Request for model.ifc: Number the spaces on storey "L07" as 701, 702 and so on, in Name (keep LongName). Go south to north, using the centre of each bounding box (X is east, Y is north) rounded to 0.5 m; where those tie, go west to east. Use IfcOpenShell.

First a look at what the model holds.

```python
import ifcopenshell
import ifcopenshell.util.element
import ifcopenshell.util.placement

model = ifcopenshell.open("model.ifc")
print(model.schema)
storey = next(s for s in model.by_type("IfcBuildingStorey") if s.Name == "L07")
spaces = [e for e in ifcopenshell.util.element.get_decomposition(storey) if e.is_a("IfcSpace")]
for e in sorted(spaces, key=lambda e: e.id()):
    origin = ifcopenshell.util.placement.get_local_placement(e.ObjectPlacement)[:3, 3]
    print(e.id(), e.Name, e.LongName, origin.round(2) + 0.0, sep=" | ")
```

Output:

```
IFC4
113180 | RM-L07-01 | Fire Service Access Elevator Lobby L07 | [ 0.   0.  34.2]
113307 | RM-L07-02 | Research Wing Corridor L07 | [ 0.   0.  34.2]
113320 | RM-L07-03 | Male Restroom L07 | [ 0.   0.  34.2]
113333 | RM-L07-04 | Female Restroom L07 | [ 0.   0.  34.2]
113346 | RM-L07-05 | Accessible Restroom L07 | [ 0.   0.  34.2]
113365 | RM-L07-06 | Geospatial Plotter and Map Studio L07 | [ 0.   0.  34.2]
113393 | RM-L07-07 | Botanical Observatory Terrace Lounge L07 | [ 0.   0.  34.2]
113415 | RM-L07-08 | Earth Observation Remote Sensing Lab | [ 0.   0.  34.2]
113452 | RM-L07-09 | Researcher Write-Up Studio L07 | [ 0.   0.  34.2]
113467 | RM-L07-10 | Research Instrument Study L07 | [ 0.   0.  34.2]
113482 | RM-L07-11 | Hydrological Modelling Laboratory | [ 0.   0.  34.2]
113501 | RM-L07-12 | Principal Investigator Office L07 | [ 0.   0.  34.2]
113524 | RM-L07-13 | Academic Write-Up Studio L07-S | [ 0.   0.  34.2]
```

```python
import ifcopenshell
import ifcopenshell.geom
import ifcopenshell.util.element
import ifcopenshell.util.shape

model = ifcopenshell.open("model.ifc")
settings = ifcopenshell.geom.settings()
settings.set("use-world-coords", True)


def centre(element):
    shape = ifcopenshell.geom.create_shape(settings, element)
    return ifcopenshell.util.shape.get_bbox_centroid(shape.geometry)


storey = next(s for s in model.by_type("IfcBuildingStorey") if s.Name == "L07")
spaces = [e for e in ifcopenshell.util.element.get_decomposition(storey) if e.is_a("IfcSpace")]

# Insertion points can sit at a corner or the storey origin, so sort by the geometry (in metres).
centres = {e: centre(e) for e in spaces}
spaces.sort(key=lambda e: (round(centres[e][1] / 0.5), centres[e][0]))

for i, e in enumerate(spaces, start=1):
    number = f"7{i:02d}"
    e.Name = number
    print(e.id(), number)

model.write("model_edited.ifc")
```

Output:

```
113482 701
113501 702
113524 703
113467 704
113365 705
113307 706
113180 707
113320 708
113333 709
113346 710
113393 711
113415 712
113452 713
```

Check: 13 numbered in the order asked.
